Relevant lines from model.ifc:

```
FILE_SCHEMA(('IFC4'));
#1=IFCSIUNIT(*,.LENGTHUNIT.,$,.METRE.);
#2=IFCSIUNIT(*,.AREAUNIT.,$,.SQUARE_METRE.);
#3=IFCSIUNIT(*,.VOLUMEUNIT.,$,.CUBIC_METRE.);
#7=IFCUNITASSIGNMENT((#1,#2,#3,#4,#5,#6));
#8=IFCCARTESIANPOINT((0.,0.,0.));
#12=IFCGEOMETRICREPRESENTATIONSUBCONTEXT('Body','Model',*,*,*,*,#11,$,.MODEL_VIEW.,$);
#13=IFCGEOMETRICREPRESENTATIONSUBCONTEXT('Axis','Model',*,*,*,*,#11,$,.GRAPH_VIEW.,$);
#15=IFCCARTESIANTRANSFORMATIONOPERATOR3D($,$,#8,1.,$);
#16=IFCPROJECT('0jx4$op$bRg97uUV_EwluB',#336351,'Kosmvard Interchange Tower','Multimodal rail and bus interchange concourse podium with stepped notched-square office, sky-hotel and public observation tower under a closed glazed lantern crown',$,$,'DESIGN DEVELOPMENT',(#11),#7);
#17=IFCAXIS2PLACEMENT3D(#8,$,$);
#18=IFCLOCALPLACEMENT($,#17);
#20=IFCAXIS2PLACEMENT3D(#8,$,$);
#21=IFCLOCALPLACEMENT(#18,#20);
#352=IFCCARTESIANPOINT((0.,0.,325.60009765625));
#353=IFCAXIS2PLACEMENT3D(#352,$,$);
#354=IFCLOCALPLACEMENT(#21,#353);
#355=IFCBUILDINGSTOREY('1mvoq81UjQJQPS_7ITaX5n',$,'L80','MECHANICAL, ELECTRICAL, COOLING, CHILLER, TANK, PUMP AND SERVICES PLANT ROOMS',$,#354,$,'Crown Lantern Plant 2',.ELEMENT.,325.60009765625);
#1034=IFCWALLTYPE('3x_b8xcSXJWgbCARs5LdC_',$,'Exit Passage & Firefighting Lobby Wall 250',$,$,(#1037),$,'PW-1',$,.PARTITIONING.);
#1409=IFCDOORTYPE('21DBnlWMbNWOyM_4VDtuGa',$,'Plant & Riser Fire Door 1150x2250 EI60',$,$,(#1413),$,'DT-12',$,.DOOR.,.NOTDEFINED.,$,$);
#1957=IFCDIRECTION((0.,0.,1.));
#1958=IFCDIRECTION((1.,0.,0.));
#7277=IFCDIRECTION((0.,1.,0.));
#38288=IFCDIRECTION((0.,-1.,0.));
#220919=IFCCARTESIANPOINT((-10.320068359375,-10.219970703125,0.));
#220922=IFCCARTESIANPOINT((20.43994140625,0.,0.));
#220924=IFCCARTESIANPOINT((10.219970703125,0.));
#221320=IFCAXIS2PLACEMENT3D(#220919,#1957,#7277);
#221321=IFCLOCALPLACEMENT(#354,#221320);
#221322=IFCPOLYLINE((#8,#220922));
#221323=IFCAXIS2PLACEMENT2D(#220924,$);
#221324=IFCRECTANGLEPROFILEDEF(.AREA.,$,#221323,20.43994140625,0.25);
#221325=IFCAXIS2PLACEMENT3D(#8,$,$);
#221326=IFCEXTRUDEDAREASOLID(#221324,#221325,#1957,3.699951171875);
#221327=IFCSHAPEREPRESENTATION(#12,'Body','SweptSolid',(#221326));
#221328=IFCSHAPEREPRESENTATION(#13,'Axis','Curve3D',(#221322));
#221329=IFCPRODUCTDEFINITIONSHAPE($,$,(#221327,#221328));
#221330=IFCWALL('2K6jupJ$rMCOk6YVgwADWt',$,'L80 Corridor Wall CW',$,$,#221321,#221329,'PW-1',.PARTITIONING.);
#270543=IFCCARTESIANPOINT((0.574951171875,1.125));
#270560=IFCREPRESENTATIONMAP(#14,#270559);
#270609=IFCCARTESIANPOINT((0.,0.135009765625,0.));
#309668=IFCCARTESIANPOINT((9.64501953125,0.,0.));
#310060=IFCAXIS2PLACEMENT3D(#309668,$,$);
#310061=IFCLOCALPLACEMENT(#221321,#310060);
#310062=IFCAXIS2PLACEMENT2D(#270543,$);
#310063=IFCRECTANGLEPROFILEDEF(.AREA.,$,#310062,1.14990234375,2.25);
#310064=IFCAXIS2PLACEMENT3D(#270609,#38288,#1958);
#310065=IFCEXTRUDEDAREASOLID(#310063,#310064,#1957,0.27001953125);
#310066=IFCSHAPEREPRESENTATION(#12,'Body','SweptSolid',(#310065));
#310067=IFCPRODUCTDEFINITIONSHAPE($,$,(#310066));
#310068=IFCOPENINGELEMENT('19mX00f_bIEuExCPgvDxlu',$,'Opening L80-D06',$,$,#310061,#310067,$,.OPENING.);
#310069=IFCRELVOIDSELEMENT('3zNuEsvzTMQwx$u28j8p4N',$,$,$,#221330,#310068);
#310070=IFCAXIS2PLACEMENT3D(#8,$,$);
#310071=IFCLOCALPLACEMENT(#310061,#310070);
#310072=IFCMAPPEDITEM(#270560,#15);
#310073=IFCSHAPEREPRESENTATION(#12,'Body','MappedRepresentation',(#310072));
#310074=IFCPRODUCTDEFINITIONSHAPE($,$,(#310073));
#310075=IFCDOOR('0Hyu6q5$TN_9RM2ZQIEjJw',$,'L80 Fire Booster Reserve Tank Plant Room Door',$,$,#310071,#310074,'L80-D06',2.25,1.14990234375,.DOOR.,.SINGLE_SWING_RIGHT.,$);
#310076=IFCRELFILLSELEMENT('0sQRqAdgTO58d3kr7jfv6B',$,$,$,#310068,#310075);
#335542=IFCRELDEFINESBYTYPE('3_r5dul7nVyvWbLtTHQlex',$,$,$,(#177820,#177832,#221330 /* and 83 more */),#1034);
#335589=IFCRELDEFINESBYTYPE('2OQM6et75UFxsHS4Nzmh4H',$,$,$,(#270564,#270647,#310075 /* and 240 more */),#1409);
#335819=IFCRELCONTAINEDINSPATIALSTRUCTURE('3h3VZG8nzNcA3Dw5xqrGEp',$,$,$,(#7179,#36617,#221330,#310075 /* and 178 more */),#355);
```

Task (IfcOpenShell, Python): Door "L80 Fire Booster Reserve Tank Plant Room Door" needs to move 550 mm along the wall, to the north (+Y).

```python
import ifcopenshell
import ifcopenshell.api.geometry
import ifcopenshell.util.placement
import ifcopenshell.util.unit

model = ifcopenshell.open("model.ifc")
unit_scale = ifcopenshell.util.unit.calculate_unit_scale(model)

door = model.by_guid("0Hyu6q5$TN_9RM2ZQIEjJw")
opening = door.FillsVoids[0].RelatingOpeningElement
wall = opening.VoidsElements[0].RelatingBuildingElement

wall_matrix = ifcopenshell.util.placement.get_local_placement(wall.ObjectPlacement)
shift = wall_matrix[:3, 0] * 0.55 / unit_scale
before = ifcopenshell.util.placement.get_local_placement(door.ObjectPlacement)[:3, 3].copy()

# The door is placed relative to its opening, so it follows when the opening moves.
matrix = ifcopenshell.util.placement.get_local_placement(opening.ObjectPlacement)
matrix[:3, 3] += shift
ifcopenshell.api.geometry.edit_object_placement(
    model, product=opening, matrix=matrix, is_si=False, should_transform_children=True
)

after = ifcopenshell.util.placement.get_local_placement(door.ObjectPlacement)[:3, 3]
print("door moved by", (after - before).round(3) + 0.0)

model.write("model_updated.ifc")
```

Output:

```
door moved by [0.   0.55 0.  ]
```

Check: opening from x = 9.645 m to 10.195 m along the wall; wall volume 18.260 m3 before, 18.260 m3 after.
